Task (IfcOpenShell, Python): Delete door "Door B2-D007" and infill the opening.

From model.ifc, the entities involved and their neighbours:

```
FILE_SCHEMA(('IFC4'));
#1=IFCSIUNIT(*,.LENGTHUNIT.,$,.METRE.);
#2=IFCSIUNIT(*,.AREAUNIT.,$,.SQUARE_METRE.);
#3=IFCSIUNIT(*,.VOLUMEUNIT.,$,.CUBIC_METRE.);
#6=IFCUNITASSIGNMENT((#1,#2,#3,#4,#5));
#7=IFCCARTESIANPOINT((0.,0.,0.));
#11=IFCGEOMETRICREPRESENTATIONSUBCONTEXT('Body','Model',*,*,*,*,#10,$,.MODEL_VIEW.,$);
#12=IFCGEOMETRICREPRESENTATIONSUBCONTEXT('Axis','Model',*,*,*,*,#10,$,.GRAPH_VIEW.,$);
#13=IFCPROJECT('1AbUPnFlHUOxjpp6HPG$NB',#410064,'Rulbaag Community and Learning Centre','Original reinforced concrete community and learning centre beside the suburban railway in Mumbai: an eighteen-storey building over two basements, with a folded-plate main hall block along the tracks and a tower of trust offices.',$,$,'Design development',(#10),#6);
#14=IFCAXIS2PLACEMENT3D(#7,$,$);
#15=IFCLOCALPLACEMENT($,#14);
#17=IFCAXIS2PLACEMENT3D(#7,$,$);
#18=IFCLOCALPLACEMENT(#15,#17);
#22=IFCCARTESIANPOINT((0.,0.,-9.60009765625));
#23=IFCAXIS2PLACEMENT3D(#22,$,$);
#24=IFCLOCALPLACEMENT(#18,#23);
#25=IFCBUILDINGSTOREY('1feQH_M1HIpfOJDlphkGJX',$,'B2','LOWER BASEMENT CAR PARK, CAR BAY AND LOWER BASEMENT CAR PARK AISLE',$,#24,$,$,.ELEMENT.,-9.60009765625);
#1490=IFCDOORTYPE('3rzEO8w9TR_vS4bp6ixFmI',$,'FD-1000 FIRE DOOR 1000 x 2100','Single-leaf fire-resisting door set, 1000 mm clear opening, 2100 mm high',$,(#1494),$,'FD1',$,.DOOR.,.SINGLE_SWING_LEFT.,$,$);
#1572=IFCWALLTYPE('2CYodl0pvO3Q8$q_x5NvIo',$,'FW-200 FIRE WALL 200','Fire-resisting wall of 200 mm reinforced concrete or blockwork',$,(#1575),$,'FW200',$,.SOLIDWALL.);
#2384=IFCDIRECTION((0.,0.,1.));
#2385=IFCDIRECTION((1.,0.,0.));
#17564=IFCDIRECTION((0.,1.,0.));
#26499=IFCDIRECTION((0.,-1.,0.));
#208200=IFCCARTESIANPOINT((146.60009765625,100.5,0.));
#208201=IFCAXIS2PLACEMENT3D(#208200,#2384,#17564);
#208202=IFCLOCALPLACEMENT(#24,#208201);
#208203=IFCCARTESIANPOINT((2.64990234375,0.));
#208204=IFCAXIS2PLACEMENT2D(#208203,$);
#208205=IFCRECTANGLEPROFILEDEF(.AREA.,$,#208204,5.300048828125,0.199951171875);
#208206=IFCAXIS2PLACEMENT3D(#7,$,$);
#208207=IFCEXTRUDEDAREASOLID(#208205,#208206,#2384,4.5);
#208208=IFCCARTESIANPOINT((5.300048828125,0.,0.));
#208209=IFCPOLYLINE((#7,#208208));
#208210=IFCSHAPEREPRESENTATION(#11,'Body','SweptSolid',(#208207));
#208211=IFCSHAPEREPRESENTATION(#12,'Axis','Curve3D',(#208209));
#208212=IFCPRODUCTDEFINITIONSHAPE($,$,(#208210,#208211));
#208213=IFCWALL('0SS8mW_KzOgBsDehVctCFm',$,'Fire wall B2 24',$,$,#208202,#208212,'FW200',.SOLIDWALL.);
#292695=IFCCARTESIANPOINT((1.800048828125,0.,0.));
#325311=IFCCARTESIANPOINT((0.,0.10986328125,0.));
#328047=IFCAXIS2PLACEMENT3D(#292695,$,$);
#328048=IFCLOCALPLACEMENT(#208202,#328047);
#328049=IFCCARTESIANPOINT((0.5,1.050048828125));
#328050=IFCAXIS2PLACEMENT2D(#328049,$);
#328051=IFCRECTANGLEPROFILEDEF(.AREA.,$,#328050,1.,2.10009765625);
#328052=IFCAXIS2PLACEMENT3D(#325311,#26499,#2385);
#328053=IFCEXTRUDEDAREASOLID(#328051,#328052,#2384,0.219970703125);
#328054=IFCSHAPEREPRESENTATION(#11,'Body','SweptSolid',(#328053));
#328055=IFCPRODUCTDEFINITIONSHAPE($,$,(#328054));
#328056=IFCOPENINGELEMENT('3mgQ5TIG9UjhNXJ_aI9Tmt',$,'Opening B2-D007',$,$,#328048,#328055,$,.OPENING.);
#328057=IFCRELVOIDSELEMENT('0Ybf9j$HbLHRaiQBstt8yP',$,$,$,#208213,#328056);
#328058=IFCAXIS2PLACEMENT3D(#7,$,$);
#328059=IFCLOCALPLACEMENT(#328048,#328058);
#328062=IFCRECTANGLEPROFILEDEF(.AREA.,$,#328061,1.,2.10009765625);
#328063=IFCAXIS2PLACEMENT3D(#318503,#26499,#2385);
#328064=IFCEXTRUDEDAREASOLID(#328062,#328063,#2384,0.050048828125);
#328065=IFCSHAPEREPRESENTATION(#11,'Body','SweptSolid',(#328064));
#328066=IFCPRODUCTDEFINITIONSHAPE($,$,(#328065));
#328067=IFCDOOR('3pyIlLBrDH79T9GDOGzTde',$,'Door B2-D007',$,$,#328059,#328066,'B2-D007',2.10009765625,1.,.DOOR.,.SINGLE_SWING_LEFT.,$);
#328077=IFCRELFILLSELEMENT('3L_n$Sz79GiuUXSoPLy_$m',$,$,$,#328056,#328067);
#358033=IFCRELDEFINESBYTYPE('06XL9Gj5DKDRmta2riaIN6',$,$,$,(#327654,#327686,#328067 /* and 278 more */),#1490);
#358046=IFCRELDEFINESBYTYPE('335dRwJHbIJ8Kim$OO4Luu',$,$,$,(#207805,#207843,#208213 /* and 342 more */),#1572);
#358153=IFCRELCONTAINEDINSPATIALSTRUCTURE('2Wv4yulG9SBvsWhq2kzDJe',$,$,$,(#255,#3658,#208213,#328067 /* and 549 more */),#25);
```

```python
import ifcopenshell
import ifcopenshell.api.feature
import ifcopenshell.api.root
import ifcopenshell.geom
import ifcopenshell.util.shape

model = ifcopenshell.open("model.ifc")
settings = ifcopenshell.geom.settings()


def volume(element):
    """Net volume in cubic metres, openings subtracted."""
    shape = ifcopenshell.geom.create_shape(settings, element)
    return ifcopenshell.util.shape.get_volume(shape.geometry)


door = model.by_guid("3pyIlLBrDH79T9GDOGzTde")
opening = door.FillsVoids[0].RelatingOpeningElement
wall = opening.VoidsElements[0].RelatingBuildingElement
before = volume(wall)

ifcopenshell.api.root.remove_product(model, product=door)
ifcopenshell.api.feature.remove_feature(model, feature=opening)

after = volume(wall)

print(f"wall volume {before:.3f} -> {after:.3f} m3")

model.write("model_rev.ifc")
```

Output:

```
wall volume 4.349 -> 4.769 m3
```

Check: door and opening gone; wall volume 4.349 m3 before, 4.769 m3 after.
